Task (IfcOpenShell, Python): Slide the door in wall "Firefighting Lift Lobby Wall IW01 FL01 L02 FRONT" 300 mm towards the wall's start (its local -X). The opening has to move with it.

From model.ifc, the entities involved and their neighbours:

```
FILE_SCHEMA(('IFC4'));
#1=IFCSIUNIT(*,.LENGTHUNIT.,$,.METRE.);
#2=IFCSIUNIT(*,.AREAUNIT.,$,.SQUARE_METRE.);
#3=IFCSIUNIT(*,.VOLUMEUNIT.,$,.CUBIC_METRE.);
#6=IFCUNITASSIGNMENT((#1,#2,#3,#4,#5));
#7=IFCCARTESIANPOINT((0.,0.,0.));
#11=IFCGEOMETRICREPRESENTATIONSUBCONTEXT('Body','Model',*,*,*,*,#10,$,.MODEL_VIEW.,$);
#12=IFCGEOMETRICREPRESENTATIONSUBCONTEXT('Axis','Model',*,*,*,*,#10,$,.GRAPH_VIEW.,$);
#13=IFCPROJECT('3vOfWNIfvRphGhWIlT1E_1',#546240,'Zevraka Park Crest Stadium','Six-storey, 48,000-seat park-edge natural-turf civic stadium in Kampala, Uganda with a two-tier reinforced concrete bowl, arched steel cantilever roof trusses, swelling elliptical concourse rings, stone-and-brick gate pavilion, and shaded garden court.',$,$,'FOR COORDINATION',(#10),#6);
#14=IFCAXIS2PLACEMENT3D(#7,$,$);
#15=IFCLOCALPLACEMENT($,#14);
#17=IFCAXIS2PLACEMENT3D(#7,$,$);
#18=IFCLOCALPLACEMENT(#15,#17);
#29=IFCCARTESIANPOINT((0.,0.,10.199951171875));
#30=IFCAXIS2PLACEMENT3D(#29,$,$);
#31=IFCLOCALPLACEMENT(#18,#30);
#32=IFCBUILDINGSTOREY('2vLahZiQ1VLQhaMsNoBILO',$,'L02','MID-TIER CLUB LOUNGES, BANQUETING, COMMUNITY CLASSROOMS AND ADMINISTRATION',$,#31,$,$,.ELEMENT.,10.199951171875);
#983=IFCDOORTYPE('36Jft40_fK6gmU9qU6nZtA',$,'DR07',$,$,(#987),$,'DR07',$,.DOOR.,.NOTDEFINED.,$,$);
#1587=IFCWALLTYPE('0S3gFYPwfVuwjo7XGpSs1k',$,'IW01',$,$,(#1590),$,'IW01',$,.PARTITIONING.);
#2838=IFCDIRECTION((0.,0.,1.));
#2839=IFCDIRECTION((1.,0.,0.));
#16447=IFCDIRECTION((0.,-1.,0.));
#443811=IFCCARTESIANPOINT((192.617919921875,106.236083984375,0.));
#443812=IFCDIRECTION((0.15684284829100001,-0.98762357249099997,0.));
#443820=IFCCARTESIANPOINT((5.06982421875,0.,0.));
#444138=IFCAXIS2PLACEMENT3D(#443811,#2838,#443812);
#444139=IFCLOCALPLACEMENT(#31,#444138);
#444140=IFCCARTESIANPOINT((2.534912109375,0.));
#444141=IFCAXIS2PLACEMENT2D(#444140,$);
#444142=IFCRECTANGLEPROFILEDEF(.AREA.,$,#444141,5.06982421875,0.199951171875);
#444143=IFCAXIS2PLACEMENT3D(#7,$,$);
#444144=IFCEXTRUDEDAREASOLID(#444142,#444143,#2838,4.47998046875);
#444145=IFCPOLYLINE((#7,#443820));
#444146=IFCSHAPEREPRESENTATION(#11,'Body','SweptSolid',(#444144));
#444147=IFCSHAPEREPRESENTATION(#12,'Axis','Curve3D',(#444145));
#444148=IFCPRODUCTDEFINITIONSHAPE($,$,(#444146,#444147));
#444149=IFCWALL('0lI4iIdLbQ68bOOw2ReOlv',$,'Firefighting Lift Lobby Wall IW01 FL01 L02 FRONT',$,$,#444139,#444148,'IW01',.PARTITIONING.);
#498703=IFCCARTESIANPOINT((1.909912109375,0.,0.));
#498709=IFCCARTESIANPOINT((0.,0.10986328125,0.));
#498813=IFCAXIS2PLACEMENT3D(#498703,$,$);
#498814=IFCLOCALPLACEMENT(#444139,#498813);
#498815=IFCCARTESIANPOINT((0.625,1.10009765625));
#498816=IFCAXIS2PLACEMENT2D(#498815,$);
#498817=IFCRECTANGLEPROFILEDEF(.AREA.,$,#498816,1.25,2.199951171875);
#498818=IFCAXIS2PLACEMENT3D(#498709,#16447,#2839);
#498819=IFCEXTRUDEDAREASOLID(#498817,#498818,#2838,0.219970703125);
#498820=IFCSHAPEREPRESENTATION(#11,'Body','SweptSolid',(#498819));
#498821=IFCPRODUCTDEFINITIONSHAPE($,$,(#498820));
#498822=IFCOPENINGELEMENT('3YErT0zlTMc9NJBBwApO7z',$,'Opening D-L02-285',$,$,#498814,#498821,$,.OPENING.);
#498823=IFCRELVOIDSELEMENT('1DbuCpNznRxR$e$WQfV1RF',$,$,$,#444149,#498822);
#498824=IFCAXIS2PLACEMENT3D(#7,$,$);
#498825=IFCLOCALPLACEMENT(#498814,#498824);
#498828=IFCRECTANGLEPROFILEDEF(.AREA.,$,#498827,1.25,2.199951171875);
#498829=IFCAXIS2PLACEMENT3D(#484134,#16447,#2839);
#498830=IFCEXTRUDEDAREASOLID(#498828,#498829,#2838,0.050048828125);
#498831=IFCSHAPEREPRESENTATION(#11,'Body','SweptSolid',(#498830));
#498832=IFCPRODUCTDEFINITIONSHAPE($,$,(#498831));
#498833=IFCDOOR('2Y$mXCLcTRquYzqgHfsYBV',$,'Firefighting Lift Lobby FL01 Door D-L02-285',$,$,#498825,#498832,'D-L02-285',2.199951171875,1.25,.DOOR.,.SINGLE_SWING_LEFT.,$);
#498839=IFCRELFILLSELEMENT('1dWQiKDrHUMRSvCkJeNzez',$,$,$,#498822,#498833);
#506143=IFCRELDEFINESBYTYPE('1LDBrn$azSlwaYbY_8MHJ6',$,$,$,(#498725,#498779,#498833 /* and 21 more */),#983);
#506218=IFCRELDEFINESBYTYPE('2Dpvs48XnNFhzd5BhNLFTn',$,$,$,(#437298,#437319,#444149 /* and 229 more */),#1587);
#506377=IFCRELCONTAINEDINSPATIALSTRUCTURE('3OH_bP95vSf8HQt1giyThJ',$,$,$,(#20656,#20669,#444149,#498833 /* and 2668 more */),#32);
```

```python
import ifcopenshell
import ifcopenshell.api.geometry
import ifcopenshell.util.placement

model = ifcopenshell.open("model.ifc")

door = model.by_id(498833)
opening = door.FillsVoids[0].RelatingOpeningElement
wall = opening.VoidsElements[0].RelatingBuildingElement

wall_matrix = ifcopenshell.util.placement.get_local_placement(wall.ObjectPlacement)
shift = wall_matrix[:3, 0] * -0.3
before = ifcopenshell.util.placement.get_local_placement(door.ObjectPlacement)[:3, 3].copy()

# The door is placed relative to its opening, so it follows when the opening moves.
matrix = ifcopenshell.util.placement.get_local_placement(opening.ObjectPlacement)
matrix[:3, 3] += shift
ifcopenshell.api.geometry.edit_object_placement(
    model, product=opening, matrix=matrix, is_si=False, should_transform_children=True
)

after = ifcopenshell.util.placement.get_local_placement(door.ObjectPlacement)[:3, 3]
print("door moved by", (after - before).round(3) + 0.0)

model.write("model_updated.ifc")
```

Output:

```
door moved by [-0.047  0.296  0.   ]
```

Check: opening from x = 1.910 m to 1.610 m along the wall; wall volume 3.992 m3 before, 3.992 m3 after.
